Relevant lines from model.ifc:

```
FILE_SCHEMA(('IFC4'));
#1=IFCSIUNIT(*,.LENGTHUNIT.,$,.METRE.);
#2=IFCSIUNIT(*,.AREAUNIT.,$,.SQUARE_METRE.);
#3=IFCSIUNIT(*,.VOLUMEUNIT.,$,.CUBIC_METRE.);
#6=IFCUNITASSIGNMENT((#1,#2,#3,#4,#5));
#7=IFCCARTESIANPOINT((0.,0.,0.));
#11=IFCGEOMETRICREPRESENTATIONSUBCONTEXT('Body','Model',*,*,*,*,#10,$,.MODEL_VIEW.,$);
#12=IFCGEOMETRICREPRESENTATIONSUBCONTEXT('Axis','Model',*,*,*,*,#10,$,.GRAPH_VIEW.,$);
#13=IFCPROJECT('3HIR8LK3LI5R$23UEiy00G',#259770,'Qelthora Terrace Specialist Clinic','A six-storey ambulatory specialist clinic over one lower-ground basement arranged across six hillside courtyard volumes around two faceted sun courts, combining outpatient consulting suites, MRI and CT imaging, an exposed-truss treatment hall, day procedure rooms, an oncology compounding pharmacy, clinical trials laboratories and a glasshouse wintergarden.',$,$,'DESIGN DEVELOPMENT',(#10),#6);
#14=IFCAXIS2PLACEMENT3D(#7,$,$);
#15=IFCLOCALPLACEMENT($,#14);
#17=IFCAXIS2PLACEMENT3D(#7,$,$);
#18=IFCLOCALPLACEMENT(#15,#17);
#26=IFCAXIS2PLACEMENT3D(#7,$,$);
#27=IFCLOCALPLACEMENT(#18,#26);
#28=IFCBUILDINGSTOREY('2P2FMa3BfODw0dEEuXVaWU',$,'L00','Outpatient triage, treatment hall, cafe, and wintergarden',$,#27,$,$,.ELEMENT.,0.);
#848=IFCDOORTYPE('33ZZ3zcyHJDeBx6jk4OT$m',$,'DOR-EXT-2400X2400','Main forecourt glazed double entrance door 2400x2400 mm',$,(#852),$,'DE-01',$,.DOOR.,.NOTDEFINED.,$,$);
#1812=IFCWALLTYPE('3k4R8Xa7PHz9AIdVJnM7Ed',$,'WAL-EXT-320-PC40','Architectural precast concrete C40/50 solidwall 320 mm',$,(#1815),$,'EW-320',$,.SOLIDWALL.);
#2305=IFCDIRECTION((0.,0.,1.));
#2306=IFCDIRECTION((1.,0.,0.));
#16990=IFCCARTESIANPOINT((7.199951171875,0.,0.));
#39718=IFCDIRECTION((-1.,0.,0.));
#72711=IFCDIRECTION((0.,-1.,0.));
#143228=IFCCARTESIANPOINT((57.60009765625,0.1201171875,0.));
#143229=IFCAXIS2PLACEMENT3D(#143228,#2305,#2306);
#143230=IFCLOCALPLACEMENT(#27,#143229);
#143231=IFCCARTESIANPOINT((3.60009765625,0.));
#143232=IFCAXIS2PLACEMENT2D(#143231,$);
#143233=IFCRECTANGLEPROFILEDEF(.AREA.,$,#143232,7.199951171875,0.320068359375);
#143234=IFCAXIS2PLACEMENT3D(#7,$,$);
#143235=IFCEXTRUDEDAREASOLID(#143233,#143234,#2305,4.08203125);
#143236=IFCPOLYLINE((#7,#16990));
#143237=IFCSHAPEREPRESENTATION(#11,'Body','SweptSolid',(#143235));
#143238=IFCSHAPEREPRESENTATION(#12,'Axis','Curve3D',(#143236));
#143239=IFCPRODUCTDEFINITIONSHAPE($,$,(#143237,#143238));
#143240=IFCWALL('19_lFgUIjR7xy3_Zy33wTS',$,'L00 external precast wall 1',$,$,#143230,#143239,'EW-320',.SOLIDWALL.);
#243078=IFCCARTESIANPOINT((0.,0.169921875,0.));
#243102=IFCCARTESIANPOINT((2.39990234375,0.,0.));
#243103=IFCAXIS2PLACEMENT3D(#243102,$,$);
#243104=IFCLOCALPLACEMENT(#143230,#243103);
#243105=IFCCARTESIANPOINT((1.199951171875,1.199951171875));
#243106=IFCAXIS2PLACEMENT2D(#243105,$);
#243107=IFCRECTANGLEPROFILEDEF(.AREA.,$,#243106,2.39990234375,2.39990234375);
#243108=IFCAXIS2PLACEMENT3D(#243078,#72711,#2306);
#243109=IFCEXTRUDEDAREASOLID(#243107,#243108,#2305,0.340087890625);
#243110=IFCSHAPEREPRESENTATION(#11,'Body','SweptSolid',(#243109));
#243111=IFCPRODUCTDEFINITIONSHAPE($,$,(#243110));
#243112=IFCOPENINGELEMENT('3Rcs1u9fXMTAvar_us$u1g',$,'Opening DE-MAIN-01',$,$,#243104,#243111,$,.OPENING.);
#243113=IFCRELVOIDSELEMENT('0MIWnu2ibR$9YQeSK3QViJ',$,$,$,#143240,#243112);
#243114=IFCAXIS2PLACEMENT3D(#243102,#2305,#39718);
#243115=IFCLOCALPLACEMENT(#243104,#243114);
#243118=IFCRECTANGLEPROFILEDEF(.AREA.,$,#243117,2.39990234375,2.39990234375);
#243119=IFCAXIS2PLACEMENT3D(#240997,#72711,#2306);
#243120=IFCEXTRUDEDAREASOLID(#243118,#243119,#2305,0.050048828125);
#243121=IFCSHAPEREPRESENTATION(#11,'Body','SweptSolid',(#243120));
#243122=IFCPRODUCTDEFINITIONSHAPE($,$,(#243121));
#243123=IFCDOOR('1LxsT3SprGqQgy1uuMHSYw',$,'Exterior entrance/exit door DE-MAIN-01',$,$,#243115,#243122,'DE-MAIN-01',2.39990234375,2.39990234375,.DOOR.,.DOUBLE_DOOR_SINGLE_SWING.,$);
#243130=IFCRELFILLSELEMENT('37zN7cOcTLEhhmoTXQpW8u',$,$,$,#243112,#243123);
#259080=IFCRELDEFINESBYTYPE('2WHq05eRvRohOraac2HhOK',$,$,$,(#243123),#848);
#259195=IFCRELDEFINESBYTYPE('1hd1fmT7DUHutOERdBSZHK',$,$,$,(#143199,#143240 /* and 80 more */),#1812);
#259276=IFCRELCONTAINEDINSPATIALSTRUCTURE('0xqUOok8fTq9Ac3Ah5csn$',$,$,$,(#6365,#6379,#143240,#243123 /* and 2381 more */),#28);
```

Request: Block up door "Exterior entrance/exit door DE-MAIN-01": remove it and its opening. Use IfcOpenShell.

```python
import ifcopenshell
import ifcopenshell.api.feature
import ifcopenshell.api.root
import ifcopenshell.geom
import ifcopenshell.util.shape

model = ifcopenshell.open("model.ifc")
settings = ifcopenshell.geom.settings()


def volume(element):
    """Net volume in cubic metres, openings subtracted."""
    shape = ifcopenshell.geom.create_shape(settings, element)
    return ifcopenshell.util.shape.get_volume(shape.geometry)


door = model.by_id(243123)
opening = door.FillsVoids[0].RelatingOpeningElement
wall = opening.VoidsElements[0].RelatingBuildingElement
before = volume(wall)

ifcopenshell.api.root.remove_product(model, product=door)
ifcopenshell.api.feature.remove_feature(model, feature=opening)

after = volume(wall)

print(f"wall volume {before:.3f} -> {after:.3f} m3")

model.write("model_rev.ifc")
```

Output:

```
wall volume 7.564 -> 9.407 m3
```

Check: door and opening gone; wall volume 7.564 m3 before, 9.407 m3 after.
